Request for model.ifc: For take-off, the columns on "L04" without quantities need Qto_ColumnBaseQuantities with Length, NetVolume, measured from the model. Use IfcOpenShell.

First a look at what the model holds.

```python
import ifcopenshell
import ifcopenshell.util.element
import ifcopenshell.util.unit

model = ifcopenshell.open("model.ifc")
print(model.schema)
for unit_type in ("LENGTHUNIT", "AREAUNIT", "VOLUMEUNIT"):
    print(unit_type, ifcopenshell.util.unit.calculate_unit_scale(model, unit_type))
storey = next(s for s in model.by_type("IfcBuildingStorey") if s.Name == "L04")
columns = [e for e in ifcopenshell.util.element.get_decomposition(storey) if e.is_a("IfcColumn")]
for e in sorted(columns, key=lambda e: e.id()):
    print(e.id(), e.is_a(), e.Name, list(ifcopenshell.util.element.get_psets(e, qtos_only=True)), sep=" | ")
```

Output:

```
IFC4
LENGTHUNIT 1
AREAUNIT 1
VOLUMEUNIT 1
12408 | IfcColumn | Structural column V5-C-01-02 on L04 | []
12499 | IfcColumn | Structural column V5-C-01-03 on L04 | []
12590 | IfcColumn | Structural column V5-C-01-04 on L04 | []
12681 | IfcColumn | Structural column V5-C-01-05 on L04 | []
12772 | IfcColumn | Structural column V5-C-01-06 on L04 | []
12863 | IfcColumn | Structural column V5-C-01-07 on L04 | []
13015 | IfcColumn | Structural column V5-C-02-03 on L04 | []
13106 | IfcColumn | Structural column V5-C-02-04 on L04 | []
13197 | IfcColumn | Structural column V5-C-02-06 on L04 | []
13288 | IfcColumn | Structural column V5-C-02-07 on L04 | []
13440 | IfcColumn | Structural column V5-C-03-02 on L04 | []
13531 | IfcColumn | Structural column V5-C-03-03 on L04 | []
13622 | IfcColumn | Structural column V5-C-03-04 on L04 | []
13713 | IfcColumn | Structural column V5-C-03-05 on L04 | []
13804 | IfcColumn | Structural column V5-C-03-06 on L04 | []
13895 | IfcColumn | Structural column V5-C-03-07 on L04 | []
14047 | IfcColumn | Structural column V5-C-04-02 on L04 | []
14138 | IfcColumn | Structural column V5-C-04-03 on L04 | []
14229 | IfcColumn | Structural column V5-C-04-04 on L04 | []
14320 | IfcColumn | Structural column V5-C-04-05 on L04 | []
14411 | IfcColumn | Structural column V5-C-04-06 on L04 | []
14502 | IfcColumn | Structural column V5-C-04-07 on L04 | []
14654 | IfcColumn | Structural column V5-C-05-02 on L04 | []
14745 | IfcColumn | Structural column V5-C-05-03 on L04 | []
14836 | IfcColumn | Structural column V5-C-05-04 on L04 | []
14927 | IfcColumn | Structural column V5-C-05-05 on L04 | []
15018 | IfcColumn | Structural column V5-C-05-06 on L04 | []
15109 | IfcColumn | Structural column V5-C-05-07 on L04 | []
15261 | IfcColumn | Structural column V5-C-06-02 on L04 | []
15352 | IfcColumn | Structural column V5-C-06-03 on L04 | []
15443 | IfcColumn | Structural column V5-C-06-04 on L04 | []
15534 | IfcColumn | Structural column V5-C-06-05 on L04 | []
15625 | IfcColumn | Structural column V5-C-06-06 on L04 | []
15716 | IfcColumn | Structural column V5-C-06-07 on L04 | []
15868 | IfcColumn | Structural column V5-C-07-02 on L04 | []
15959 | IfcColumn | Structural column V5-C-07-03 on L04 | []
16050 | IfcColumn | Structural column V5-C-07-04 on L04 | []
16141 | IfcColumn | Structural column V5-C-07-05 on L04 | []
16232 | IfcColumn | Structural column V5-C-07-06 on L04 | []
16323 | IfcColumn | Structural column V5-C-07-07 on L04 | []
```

```python
import ifcopenshell
import ifcopenshell.api.pset
import ifcopenshell.geom
import ifcopenshell.util.element
import ifcopenshell.util.shape
import ifcopenshell.util.unit

model = ifcopenshell.open("model.ifc")
unit_scale = ifcopenshell.util.unit.calculate_unit_scale(model)
volume_scale = ifcopenshell.util.unit.calculate_unit_scale(model, "VOLUMEUNIT")
settings = ifcopenshell.geom.settings()

storey = next(s for s in model.by_type("IfcBuildingStorey") if s.Name == "L04")
columns = [e for e in ifcopenshell.util.element.get_decomposition(storey) if e.is_a("IfcColumn")]

for e in sorted(columns, key=lambda e: e.id()):
    if ifcopenshell.util.element.get_psets(e, qtos_only=True, should_inherit=False):
        continue
    # Geometry comes back in metres, in the element's own axes.
    shape = ifcopenshell.geom.create_shape(settings, e)
    values = {
        "Length": ifcopenshell.util.shape.get_z(shape.geometry) / unit_scale,
        "NetVolume": ifcopenshell.util.shape.get_volume(shape.geometry) / volume_scale,
    }
    qto = ifcopenshell.api.pset.add_qto(model, product=e, name="Qto_ColumnBaseQuantities")
    ifcopenshell.api.pset.edit_qto(model, qto=qto, properties=values)
    print(e.id(), {k: round(v, 3) for k, v in values.items()})

model.write("model_v2.ifc")
```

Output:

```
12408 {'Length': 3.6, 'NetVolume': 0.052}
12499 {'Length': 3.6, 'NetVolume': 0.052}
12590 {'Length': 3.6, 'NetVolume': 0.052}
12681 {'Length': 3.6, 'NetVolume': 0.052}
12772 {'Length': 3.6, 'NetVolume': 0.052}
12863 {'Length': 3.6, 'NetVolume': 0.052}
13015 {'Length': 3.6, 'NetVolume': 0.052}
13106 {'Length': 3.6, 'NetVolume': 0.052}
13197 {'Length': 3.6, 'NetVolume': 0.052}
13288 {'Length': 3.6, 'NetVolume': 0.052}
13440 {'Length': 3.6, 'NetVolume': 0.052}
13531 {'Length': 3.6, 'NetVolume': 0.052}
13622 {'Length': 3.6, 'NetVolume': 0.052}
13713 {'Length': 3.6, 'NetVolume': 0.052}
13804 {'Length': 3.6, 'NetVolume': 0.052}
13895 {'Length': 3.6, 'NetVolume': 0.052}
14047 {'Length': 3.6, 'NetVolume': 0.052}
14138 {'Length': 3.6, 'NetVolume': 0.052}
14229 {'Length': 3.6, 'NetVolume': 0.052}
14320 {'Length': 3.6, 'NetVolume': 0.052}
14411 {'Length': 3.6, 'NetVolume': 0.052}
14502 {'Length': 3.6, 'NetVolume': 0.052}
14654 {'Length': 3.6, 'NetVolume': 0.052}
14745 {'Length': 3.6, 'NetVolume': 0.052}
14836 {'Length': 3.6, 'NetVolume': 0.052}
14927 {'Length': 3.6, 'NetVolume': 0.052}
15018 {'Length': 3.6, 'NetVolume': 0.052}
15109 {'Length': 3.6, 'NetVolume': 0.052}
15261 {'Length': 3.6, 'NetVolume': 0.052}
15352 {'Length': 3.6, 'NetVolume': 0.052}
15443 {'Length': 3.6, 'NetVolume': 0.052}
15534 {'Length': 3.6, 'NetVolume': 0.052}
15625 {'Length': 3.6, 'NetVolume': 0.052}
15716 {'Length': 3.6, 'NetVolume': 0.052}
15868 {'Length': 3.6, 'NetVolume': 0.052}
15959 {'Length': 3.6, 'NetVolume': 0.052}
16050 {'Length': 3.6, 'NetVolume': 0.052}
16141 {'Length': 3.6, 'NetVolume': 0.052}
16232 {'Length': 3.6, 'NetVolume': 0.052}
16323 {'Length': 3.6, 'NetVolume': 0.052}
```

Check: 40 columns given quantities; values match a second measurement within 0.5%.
